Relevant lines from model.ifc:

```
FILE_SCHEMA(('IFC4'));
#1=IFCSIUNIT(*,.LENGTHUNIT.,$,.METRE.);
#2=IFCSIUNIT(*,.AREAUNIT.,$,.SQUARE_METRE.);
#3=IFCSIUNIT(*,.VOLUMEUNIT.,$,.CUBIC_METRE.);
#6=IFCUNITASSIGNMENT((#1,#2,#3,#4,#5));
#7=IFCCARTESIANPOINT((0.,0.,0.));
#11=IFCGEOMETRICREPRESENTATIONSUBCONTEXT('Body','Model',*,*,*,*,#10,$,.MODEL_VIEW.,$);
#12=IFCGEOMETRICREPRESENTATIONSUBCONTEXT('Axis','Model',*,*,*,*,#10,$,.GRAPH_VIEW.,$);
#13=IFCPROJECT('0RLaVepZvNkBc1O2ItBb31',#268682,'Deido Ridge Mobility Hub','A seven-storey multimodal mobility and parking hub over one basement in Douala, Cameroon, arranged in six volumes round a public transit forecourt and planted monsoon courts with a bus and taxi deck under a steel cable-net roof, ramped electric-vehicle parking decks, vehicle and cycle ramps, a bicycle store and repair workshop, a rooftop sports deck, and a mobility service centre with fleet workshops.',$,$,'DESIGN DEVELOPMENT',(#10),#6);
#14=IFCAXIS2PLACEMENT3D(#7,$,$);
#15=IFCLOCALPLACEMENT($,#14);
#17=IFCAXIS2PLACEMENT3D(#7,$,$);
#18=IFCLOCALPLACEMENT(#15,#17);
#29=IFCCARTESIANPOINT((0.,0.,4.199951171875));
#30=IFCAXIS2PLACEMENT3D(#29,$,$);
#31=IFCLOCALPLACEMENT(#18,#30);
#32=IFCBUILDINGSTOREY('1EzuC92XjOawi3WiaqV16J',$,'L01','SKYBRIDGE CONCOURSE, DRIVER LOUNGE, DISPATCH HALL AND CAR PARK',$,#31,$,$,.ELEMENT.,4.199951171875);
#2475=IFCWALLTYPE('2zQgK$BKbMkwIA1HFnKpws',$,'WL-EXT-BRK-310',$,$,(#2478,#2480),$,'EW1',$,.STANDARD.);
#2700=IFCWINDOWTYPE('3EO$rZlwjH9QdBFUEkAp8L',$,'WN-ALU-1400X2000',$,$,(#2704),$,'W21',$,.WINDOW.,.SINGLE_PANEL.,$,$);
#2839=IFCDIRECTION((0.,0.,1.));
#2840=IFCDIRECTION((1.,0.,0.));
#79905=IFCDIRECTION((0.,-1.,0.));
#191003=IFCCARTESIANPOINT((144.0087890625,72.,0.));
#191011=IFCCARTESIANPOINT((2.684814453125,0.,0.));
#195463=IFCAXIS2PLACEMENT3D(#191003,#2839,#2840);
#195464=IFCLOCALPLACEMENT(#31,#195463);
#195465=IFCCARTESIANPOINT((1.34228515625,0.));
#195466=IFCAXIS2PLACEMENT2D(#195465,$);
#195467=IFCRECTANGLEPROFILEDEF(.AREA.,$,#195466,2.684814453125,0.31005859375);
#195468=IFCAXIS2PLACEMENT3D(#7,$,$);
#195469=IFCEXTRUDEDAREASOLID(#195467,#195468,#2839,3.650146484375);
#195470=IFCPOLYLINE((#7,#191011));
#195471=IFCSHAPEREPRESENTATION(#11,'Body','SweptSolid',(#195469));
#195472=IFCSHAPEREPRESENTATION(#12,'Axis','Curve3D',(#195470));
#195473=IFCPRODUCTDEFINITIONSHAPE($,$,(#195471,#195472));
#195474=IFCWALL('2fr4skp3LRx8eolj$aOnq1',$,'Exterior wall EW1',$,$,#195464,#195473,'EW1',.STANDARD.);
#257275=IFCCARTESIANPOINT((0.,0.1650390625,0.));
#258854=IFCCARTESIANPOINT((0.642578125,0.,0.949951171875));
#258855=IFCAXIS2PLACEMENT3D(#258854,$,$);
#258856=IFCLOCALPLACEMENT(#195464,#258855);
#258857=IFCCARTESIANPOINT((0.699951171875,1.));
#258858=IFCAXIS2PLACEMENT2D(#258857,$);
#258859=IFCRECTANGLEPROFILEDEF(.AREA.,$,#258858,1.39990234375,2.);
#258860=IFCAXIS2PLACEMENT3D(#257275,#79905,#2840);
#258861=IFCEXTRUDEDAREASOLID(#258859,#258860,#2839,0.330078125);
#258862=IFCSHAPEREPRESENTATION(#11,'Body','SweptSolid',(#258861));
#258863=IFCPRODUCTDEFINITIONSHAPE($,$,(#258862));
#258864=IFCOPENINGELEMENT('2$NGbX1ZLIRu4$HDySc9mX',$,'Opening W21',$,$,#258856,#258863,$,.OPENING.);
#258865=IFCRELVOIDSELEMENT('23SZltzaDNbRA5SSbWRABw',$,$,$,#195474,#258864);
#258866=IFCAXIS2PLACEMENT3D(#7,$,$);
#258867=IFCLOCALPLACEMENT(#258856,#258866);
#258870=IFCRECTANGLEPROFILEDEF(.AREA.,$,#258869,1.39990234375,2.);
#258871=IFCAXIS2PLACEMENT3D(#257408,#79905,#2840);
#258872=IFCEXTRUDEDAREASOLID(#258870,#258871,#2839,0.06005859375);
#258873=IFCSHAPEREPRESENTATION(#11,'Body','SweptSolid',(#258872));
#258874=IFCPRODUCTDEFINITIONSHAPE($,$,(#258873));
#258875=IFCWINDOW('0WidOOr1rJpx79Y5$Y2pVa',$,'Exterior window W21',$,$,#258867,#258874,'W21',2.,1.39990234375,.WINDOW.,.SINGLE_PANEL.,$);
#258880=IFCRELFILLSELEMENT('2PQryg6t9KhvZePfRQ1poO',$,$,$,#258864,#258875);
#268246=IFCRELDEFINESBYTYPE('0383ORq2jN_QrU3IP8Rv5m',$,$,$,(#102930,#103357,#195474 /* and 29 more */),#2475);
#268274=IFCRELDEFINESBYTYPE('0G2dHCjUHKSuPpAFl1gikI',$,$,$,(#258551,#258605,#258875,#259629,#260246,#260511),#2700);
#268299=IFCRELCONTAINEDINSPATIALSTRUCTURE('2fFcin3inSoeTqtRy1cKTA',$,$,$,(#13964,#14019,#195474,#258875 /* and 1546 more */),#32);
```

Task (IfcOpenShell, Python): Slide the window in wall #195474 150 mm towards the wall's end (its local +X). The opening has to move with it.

```python
import ifcopenshell
import ifcopenshell.api.geometry
import ifcopenshell.util.placement
import ifcopenshell.util.unit

model = ifcopenshell.open("model.ifc")
unit_scale = ifcopenshell.util.unit.calculate_unit_scale(model)

window = model.by_guid("0WidOOr1rJpx79Y5$Y2pVa")
opening = window.FillsVoids[0].RelatingOpeningElement
wall = opening.VoidsElements[0].RelatingBuildingElement

wall_matrix = ifcopenshell.util.placement.get_local_placement(wall.ObjectPlacement)
shift = wall_matrix[:3, 0] * 0.15 / unit_scale
before = ifcopenshell.util.placement.get_local_placement(window.ObjectPlacement)[:3, 3].copy()

# The window is placed relative to its opening, so it follows when the opening moves.
matrix = ifcopenshell.util.placement.get_local_placement(opening.ObjectPlacement)
matrix[:3, 3] += shift
ifcopenshell.api.geometry.edit_object_placement(
    model, product=opening, matrix=matrix, is_si=False, should_transform_children=True
)

after = ifcopenshell.util.placement.get_local_placement(window.ObjectPlacement)[:3, 3]
print("window moved by", (after - before).round(3) + 0.0)

model.write("model_updated.ifc")
```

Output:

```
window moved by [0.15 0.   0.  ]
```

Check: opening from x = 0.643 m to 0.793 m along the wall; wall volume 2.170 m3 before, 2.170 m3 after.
